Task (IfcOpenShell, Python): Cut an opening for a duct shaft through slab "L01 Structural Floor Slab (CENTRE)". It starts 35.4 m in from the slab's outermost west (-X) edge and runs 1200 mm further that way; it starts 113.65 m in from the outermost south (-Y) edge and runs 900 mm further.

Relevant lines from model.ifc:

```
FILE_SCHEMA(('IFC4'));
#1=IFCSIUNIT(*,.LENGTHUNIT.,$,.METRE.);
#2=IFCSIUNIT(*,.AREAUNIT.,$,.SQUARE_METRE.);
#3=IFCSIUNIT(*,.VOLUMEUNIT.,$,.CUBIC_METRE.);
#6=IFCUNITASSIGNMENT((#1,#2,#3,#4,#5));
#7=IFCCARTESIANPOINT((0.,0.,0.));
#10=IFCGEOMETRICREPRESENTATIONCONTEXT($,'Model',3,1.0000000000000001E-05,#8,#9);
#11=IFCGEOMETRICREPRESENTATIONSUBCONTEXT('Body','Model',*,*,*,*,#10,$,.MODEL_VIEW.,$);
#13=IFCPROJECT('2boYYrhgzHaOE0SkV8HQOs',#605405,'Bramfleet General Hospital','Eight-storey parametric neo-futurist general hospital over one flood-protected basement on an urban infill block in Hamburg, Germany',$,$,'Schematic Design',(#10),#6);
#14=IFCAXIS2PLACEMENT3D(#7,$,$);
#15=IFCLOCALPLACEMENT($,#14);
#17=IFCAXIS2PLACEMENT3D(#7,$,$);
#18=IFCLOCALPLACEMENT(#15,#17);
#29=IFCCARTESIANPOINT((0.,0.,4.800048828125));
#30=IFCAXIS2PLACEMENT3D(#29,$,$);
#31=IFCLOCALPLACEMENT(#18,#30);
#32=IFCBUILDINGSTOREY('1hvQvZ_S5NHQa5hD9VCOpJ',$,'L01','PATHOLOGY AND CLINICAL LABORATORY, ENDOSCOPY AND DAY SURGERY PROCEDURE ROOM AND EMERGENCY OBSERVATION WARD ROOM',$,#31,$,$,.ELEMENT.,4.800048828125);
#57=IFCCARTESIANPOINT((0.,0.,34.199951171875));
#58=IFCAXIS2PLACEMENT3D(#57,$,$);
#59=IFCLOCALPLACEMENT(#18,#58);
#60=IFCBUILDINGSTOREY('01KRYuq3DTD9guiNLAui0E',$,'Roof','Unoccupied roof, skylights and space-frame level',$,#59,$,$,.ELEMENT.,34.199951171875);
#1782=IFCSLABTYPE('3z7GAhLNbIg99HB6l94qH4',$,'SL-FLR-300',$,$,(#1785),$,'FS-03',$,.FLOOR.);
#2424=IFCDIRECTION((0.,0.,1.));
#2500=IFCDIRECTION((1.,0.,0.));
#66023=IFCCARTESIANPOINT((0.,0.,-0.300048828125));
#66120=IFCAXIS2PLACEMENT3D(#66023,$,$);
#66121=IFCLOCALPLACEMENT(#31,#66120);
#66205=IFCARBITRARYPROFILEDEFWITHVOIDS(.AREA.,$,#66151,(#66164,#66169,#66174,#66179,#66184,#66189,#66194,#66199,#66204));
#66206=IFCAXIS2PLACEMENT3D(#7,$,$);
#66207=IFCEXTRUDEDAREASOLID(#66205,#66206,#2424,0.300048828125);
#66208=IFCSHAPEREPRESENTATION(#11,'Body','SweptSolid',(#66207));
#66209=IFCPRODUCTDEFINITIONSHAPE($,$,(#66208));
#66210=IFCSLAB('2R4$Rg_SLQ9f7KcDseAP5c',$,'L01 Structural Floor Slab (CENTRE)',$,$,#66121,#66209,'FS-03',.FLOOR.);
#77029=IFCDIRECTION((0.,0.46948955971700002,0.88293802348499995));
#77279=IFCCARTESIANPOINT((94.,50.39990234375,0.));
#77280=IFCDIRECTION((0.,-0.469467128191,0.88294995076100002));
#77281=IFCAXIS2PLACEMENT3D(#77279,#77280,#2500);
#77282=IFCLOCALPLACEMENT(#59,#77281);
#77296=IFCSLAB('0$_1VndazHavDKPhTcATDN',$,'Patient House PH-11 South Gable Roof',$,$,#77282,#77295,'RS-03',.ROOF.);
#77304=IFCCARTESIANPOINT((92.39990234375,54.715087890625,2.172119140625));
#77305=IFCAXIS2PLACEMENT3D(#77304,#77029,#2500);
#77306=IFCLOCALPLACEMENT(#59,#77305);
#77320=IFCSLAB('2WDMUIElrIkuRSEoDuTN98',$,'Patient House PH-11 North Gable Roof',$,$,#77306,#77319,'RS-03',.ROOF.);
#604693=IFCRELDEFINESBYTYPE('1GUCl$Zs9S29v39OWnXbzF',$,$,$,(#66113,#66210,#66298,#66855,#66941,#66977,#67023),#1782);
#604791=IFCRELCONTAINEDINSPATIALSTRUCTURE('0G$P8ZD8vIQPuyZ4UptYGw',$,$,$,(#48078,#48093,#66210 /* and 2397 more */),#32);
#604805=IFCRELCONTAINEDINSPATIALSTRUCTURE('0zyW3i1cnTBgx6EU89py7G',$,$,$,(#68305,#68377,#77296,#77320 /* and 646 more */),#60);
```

```python
import numpy as np
import ifcopenshell
import ifcopenshell.api.feature
import ifcopenshell.api.geometry
import ifcopenshell.api.root
import ifcopenshell.geom
import ifcopenshell.util.placement
import ifcopenshell.util.representation
import ifcopenshell.util.shape
import ifcopenshell.util.unit

model = ifcopenshell.open("model.ifc")
unit_scale = ifcopenshell.util.unit.calculate_unit_scale(model)
settings = ifcopenshell.geom.settings()


def volume(element):
    """Net volume in cubic metres, openings subtracted."""
    shape = ifcopenshell.geom.create_shape(settings, element)
    return ifcopenshell.util.shape.get_volume(shape.geometry)


slab = model.by_id(66210)
before = volume(slab)

# Extent in the slab's own axes, in metres. The edges named are its -X and -Y sides.
slab_shape = ifcopenshell.geom.create_shape(settings, slab)
vertices = ifcopenshell.util.shape.get_vertices(slab_shape.geometry)
x_min, y_min, bottom = vertices.min(axis=0)
top = vertices[:, 2].max()

opening = ifcopenshell.api.root.create_entity(model, ifc_class="IfcOpeningElement", name="Duct shaft opening", predefined_type="OPENING")
context = ifcopenshell.util.representation.get_context(model, "Model", "Body", "MODEL_VIEW")
width, depth = 1.2, 0.9
outline = [(0.0, 0.0), (width, 0.0), (width, depth), (0.0, depth), (0.0, 0.0)]
# Overshoot both faces by 50 mm so the cut is clean.
shape = ifcopenshell.api.geometry.add_slab_representation(
    model, context=context, depth=top - bottom + 0.1, polyline=outline
)
ifcopenshell.api.geometry.assign_representation(model, product=opening, representation=shape)

matrix = ifcopenshell.util.placement.get_local_placement(slab.ObjectPlacement)
matrix[:, 3] = matrix @ np.append(np.array([x_min + 35.4, y_min + 113.65, bottom - 0.05]) / unit_scale, 1.0)
ifcopenshell.api.geometry.edit_object_placement(model, product=opening, matrix=matrix, is_si=False)
ifcopenshell.api.feature.add_feature(model, feature=opening, element=slab)

after = volume(slab)

print(f"slab volume {before:.3f} -> {after:.3f} m3")

model.write("model-out.ifc")
```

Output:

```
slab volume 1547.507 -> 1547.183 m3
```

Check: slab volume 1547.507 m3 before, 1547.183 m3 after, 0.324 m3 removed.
